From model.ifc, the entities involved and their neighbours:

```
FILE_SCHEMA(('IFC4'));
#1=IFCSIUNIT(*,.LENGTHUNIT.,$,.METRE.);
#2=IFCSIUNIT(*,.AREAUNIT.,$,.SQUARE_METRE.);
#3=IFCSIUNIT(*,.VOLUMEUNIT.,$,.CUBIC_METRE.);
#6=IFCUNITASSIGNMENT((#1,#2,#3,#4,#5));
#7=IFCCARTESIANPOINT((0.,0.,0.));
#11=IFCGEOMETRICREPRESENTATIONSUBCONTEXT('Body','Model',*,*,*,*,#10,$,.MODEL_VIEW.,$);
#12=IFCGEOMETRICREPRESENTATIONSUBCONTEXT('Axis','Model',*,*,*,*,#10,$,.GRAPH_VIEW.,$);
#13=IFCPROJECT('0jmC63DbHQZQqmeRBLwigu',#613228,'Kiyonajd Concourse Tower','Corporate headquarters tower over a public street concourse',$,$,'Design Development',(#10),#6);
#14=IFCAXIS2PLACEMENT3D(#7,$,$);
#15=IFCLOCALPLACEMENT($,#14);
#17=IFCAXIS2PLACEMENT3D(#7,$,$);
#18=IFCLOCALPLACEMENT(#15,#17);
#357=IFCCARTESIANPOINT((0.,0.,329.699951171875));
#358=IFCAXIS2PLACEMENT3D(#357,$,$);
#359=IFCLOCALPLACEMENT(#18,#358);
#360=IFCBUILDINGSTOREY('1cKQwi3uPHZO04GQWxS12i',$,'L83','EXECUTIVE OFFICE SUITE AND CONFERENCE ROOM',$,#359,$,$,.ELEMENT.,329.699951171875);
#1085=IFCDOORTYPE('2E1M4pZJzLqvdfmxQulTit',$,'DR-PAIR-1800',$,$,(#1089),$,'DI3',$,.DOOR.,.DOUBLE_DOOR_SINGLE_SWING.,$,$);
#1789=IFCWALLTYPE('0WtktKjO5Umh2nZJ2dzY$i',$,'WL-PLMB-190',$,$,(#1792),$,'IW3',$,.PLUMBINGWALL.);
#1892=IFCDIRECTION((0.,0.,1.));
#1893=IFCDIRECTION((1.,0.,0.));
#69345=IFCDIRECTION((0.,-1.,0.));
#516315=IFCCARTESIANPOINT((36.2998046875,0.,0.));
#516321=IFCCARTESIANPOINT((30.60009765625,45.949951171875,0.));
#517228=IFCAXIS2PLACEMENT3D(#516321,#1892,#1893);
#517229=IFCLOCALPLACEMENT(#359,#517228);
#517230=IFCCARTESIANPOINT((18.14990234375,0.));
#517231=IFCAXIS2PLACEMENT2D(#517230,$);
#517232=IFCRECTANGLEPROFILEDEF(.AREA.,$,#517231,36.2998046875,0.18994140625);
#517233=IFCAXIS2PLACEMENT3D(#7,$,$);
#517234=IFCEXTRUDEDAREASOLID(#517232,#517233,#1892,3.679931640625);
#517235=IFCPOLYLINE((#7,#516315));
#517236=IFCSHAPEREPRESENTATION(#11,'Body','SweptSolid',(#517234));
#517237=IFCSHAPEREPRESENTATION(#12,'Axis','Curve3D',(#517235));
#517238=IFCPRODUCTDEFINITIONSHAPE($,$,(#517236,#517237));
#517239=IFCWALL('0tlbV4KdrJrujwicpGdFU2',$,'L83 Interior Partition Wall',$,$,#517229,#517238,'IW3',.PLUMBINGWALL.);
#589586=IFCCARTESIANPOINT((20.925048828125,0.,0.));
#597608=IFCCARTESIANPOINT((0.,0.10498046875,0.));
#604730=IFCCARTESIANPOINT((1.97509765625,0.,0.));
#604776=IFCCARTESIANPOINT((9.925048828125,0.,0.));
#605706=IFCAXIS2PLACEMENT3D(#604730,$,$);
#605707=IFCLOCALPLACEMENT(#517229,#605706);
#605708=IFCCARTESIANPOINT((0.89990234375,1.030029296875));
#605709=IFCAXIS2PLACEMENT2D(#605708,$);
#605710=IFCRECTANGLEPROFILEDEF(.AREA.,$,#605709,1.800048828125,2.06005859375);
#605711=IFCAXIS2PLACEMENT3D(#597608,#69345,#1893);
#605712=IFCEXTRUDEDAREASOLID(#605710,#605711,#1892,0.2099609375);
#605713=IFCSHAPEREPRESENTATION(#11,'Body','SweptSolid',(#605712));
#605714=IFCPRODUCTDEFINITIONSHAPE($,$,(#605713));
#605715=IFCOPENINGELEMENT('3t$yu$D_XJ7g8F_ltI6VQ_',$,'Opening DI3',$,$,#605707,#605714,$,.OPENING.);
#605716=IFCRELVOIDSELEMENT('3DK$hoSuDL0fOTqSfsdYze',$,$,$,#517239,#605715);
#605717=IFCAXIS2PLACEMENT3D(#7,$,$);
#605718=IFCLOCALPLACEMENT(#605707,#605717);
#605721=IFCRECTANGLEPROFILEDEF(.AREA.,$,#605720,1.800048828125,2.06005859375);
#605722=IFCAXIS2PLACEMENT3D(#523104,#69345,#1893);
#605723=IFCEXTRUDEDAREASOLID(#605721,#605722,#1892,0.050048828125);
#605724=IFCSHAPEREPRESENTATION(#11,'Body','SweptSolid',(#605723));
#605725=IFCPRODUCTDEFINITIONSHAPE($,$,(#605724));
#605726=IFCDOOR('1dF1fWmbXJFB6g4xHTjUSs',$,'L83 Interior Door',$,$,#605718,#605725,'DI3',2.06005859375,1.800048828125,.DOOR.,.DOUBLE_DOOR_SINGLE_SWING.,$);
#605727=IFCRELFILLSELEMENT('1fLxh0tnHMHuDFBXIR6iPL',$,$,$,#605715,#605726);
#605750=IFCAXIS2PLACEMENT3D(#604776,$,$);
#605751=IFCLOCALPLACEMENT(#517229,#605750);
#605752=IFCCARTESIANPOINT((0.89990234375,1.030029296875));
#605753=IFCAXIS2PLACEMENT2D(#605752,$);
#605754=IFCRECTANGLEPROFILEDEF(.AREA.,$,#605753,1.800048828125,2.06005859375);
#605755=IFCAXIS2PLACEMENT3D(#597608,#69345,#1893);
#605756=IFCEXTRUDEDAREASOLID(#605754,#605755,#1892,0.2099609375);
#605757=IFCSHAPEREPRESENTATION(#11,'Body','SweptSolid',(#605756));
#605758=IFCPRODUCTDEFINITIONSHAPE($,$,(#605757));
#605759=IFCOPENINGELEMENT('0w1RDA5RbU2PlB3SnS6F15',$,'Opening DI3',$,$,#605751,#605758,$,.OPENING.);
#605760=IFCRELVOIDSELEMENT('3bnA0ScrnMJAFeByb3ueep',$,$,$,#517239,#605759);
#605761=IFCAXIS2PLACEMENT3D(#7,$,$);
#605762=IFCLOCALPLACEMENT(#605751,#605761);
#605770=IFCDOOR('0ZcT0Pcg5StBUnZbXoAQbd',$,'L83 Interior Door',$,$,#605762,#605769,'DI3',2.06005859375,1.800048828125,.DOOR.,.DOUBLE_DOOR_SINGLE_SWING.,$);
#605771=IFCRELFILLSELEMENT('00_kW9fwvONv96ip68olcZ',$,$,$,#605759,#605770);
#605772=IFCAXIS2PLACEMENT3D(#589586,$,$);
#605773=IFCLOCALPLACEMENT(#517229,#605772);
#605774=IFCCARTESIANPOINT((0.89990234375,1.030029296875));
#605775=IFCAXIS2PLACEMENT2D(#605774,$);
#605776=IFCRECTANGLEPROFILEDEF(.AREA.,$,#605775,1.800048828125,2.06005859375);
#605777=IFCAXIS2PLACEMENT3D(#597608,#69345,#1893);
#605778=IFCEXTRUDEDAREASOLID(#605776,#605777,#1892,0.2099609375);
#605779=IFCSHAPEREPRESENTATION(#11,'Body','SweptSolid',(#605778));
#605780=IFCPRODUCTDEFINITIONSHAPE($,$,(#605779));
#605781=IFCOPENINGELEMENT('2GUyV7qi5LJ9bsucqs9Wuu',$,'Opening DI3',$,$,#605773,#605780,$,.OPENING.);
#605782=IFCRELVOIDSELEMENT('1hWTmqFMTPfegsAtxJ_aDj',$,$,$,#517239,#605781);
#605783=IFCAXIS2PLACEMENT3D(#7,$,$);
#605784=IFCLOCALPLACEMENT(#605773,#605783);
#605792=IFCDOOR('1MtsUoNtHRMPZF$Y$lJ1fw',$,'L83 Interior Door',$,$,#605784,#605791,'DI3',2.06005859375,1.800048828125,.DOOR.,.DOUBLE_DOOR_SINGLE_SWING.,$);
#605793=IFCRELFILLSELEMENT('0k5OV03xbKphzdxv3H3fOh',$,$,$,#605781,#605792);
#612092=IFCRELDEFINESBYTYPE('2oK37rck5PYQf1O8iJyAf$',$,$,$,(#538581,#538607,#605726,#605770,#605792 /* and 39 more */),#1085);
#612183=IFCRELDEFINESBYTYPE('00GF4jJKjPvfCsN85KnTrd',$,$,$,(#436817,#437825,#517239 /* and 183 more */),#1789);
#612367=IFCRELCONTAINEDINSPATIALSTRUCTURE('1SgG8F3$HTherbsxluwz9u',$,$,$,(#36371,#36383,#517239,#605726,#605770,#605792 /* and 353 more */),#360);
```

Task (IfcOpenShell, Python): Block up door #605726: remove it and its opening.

```python
import ifcopenshell
import ifcopenshell.api.feature
import ifcopenshell.api.root
import ifcopenshell.geom
import ifcopenshell.util.shape

model = ifcopenshell.open("model.ifc")
settings = ifcopenshell.geom.settings()


def volume(element):
    """Net volume in cubic metres, openings subtracted."""
    shape = ifcopenshell.geom.create_shape(settings, element)
    return ifcopenshell.util.shape.get_volume(shape.geometry)


door = model.by_id(605726)
opening = door.FillsVoids[0].RelatingOpeningElement
wall = opening.VoidsElements[0].RelatingBuildingElement
before = volume(wall)

ifcopenshell.api.root.remove_product(model, product=door)
ifcopenshell.api.feature.remove_feature(model, feature=opening)

after = volume(wall)

print(f"wall volume {before:.3f} -> {after:.3f} m3")

model.write("model-out.ifc")
```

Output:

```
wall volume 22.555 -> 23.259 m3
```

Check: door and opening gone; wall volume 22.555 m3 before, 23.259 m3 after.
